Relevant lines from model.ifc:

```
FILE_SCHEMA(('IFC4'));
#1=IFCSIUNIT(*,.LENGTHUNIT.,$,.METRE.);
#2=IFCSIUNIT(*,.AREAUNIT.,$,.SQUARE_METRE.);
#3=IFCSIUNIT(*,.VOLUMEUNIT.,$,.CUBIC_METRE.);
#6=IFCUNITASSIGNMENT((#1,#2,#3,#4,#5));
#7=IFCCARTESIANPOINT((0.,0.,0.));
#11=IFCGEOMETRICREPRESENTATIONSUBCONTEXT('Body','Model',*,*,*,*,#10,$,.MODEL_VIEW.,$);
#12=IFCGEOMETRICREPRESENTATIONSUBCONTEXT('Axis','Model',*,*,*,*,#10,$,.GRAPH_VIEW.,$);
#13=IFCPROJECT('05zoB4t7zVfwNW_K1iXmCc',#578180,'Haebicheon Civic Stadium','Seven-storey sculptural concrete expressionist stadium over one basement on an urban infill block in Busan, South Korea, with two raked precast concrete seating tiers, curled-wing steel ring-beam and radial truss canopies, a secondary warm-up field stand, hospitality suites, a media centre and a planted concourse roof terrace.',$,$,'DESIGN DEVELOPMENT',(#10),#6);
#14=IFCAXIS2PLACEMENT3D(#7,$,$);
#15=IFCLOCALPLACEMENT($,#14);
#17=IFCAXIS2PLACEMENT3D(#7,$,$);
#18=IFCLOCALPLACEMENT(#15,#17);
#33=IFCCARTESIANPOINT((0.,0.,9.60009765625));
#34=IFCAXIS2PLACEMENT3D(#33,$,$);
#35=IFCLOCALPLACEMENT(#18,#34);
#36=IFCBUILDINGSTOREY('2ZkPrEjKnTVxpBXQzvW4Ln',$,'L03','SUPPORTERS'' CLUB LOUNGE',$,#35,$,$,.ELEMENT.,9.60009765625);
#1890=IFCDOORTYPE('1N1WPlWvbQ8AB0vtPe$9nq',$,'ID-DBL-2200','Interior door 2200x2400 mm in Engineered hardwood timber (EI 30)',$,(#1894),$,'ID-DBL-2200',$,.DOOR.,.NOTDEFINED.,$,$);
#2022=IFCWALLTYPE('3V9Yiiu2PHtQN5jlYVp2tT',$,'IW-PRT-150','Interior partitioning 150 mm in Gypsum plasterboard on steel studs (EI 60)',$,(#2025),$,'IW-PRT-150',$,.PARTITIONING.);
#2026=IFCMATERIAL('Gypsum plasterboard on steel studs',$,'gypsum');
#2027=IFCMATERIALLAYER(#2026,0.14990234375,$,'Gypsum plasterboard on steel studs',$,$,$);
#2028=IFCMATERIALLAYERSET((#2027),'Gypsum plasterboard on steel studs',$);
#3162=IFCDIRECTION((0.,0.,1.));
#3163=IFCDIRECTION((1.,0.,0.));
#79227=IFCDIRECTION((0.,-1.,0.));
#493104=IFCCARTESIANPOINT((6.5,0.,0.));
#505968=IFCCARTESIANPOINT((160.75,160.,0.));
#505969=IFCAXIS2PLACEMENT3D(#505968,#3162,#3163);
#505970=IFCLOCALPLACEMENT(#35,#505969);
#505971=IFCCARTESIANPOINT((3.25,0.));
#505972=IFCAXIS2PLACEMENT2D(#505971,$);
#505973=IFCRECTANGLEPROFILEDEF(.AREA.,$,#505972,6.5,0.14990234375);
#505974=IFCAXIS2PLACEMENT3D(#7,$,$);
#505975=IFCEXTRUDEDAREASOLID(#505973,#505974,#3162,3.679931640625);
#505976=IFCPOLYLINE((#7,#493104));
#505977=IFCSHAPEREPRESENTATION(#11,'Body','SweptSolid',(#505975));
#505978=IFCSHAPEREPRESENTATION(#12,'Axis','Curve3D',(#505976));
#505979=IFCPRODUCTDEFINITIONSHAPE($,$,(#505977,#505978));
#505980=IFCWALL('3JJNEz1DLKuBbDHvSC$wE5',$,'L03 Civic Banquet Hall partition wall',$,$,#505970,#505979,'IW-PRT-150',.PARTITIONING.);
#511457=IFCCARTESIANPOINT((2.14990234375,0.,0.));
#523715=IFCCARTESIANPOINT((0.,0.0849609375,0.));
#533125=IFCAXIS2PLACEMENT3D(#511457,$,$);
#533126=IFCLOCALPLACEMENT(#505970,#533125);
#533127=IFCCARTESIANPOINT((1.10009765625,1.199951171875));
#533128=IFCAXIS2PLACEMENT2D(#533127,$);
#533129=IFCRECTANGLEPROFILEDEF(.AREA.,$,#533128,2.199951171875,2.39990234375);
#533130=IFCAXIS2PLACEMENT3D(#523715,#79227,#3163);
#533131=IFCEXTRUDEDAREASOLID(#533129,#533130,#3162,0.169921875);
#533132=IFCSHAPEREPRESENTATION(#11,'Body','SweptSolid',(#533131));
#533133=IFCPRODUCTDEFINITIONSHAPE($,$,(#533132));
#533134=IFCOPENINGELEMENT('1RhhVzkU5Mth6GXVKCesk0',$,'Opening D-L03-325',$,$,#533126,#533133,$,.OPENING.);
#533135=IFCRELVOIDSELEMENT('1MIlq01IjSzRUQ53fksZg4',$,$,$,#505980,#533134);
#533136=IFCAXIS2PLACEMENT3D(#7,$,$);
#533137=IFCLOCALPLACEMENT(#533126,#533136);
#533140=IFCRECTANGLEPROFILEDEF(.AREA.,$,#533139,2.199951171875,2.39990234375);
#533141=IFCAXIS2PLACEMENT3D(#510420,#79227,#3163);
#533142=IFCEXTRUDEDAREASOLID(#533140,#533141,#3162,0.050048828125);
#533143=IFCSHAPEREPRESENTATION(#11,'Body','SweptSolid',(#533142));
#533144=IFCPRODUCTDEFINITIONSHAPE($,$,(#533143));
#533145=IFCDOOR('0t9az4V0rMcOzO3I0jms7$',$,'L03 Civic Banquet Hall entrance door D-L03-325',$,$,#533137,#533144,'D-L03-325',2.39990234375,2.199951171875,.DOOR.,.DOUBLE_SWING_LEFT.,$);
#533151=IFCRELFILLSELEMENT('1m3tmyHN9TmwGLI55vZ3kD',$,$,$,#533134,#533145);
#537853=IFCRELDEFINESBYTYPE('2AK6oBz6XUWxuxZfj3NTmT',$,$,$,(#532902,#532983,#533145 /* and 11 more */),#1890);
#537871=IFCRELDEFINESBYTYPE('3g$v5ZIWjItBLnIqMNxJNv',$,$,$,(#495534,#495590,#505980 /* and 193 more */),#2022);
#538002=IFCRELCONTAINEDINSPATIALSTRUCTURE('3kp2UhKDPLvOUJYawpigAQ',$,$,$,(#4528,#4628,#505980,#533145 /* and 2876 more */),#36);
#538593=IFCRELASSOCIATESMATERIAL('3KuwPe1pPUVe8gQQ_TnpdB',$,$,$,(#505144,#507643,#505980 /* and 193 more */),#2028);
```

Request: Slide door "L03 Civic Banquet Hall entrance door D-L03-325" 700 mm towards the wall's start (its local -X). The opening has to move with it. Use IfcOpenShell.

```python
import ifcopenshell
import ifcopenshell.api.geometry
import ifcopenshell.util.placement
import ifcopenshell.util.unit

model = ifcopenshell.open("model.ifc")
unit_scale = ifcopenshell.util.unit.calculate_unit_scale(model)

door = model.by_guid("0t9az4V0rMcOzO3I0jms7$")
opening = door.FillsVoids[0].RelatingOpeningElement
wall = opening.VoidsElements[0].RelatingBuildingElement

wall_matrix = ifcopenshell.util.placement.get_local_placement(wall.ObjectPlacement)
shift = wall_matrix[:3, 0] * -0.7 / unit_scale
before = ifcopenshell.util.placement.get_local_placement(door.ObjectPlacement)[:3, 3].copy()

# The door is placed relative to its opening, so it follows when the opening moves.
matrix = ifcopenshell.util.placement.get_local_placement(opening.ObjectPlacement)
matrix[:3, 3] += shift
ifcopenshell.api.geometry.edit_object_placement(
    model, product=opening, matrix=matrix, is_si=False, should_transform_children=True
)

after = ifcopenshell.util.placement.get_local_placement(door.ObjectPlacement)[:3, 3]
print("door moved by", (after - before).round(3) + 0.0)

model.write("model_edited.ifc")
```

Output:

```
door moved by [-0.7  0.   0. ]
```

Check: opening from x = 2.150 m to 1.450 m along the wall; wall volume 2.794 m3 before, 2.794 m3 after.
